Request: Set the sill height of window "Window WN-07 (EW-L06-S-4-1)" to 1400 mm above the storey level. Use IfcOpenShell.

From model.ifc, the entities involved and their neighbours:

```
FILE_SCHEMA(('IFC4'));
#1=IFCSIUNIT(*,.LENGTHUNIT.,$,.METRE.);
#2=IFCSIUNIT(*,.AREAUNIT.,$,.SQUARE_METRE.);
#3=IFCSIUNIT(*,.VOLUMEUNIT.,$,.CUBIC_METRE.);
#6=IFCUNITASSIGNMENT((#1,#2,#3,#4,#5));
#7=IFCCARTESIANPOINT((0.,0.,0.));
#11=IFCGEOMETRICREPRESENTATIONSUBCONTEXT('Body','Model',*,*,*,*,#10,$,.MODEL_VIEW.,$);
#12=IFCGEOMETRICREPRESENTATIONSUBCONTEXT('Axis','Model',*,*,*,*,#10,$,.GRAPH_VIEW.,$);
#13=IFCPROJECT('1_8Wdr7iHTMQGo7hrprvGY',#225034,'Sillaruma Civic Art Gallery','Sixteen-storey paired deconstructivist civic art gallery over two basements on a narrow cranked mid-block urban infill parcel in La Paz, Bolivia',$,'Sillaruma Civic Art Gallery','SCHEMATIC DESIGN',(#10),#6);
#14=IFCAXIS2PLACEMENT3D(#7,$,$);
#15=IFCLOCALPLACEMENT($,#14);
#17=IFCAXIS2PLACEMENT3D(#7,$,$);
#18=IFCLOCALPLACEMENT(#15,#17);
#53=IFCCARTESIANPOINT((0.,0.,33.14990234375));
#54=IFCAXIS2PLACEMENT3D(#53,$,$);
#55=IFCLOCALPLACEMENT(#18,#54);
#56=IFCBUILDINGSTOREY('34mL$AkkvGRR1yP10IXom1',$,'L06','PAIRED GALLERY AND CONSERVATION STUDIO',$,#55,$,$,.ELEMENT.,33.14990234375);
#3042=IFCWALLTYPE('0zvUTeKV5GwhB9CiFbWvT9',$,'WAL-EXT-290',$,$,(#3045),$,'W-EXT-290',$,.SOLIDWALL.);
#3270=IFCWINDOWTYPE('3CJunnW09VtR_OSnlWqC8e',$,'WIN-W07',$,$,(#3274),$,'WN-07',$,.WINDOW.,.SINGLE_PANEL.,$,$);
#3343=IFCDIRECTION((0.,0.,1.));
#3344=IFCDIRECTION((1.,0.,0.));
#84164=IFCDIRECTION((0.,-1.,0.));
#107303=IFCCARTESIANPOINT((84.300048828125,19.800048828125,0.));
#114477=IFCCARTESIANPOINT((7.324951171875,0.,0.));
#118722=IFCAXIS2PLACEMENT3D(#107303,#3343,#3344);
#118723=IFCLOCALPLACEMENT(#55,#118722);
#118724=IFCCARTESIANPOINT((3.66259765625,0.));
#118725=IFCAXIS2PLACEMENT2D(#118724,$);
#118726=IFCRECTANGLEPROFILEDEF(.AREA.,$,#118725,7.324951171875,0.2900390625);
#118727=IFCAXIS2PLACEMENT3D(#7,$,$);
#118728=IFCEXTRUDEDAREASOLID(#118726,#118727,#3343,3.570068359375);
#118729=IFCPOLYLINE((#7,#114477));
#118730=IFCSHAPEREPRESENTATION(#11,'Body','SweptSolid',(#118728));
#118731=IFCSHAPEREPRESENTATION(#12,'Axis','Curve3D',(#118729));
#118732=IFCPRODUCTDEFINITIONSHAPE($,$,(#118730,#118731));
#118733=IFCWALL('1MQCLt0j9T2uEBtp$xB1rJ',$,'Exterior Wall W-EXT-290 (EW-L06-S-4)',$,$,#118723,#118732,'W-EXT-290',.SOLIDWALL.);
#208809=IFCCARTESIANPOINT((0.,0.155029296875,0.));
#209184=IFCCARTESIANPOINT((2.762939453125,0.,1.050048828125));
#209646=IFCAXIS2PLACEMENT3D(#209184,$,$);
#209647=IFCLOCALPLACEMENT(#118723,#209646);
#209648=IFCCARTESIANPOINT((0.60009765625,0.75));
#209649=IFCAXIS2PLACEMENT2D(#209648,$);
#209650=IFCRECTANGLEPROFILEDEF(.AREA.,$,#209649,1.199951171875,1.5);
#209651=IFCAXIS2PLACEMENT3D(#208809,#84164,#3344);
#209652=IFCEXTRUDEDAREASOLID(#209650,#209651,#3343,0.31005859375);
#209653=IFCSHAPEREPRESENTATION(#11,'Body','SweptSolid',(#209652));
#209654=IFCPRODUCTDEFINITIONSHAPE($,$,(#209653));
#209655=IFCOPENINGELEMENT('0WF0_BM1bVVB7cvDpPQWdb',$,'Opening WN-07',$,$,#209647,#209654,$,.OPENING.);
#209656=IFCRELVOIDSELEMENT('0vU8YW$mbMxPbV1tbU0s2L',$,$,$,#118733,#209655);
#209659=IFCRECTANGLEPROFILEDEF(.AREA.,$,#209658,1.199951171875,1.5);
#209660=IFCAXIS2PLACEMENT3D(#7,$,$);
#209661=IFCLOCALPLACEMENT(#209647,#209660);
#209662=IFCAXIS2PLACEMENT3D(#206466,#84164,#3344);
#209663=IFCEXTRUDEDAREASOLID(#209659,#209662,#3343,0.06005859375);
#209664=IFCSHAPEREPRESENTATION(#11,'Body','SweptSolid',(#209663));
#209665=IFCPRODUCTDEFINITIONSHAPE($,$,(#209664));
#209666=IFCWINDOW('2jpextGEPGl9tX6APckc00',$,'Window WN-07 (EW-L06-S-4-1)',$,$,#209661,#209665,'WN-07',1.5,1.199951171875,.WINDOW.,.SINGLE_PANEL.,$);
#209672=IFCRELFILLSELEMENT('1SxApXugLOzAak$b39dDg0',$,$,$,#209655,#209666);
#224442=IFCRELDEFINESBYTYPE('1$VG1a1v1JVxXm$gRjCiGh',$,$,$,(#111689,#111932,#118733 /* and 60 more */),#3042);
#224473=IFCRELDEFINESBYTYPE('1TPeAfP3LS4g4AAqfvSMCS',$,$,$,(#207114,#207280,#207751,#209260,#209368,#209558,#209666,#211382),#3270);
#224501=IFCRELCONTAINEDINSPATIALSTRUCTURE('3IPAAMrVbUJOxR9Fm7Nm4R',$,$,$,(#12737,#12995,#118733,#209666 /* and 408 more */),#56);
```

```python
import numpy as np
import ifcopenshell
import ifcopenshell.api.geometry
import ifcopenshell.geom
import ifcopenshell.util.element
import ifcopenshell.util.placement
import ifcopenshell.util.shape
import ifcopenshell.util.unit

model = ifcopenshell.open("model.ifc")
unit_scale = ifcopenshell.util.unit.calculate_unit_scale(model)

window = model.by_guid("2jpextGEPGl9tX6APckc00")
opening = window.FillsVoids[0].RelatingOpeningElement
storey = ifcopenshell.util.element.get_container(window, ifc_class="IfcBuildingStorey")
level = ifcopenshell.util.placement.get_local_placement(storey.ObjectPlacement)[2, 3]

# The opening's origin need not be at the sill, so measure its lowest point.
shape = ifcopenshell.geom.create_shape(ifcopenshell.geom.settings(), opening)
bottom = ifcopenshell.util.shape.get_shape_bottom_elevation(shape, shape.geometry) / unit_scale
dz = level + 1.4 / unit_scale - bottom

shift = np.array([0.0, 0.0, dz])
# The window is placed relative to its opening, so it follows when the opening moves.
matrix = ifcopenshell.util.placement.get_local_placement(opening.ObjectPlacement)
matrix[:3, 3] += shift
ifcopenshell.api.geometry.edit_object_placement(
    model, product=opening, matrix=matrix, is_si=False, should_transform_children=True
)

print(f"moved by {dz * unit_scale:+.3f} m")

model.write("model_updated.ifc")
```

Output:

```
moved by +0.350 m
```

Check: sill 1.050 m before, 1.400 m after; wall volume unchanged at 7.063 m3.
